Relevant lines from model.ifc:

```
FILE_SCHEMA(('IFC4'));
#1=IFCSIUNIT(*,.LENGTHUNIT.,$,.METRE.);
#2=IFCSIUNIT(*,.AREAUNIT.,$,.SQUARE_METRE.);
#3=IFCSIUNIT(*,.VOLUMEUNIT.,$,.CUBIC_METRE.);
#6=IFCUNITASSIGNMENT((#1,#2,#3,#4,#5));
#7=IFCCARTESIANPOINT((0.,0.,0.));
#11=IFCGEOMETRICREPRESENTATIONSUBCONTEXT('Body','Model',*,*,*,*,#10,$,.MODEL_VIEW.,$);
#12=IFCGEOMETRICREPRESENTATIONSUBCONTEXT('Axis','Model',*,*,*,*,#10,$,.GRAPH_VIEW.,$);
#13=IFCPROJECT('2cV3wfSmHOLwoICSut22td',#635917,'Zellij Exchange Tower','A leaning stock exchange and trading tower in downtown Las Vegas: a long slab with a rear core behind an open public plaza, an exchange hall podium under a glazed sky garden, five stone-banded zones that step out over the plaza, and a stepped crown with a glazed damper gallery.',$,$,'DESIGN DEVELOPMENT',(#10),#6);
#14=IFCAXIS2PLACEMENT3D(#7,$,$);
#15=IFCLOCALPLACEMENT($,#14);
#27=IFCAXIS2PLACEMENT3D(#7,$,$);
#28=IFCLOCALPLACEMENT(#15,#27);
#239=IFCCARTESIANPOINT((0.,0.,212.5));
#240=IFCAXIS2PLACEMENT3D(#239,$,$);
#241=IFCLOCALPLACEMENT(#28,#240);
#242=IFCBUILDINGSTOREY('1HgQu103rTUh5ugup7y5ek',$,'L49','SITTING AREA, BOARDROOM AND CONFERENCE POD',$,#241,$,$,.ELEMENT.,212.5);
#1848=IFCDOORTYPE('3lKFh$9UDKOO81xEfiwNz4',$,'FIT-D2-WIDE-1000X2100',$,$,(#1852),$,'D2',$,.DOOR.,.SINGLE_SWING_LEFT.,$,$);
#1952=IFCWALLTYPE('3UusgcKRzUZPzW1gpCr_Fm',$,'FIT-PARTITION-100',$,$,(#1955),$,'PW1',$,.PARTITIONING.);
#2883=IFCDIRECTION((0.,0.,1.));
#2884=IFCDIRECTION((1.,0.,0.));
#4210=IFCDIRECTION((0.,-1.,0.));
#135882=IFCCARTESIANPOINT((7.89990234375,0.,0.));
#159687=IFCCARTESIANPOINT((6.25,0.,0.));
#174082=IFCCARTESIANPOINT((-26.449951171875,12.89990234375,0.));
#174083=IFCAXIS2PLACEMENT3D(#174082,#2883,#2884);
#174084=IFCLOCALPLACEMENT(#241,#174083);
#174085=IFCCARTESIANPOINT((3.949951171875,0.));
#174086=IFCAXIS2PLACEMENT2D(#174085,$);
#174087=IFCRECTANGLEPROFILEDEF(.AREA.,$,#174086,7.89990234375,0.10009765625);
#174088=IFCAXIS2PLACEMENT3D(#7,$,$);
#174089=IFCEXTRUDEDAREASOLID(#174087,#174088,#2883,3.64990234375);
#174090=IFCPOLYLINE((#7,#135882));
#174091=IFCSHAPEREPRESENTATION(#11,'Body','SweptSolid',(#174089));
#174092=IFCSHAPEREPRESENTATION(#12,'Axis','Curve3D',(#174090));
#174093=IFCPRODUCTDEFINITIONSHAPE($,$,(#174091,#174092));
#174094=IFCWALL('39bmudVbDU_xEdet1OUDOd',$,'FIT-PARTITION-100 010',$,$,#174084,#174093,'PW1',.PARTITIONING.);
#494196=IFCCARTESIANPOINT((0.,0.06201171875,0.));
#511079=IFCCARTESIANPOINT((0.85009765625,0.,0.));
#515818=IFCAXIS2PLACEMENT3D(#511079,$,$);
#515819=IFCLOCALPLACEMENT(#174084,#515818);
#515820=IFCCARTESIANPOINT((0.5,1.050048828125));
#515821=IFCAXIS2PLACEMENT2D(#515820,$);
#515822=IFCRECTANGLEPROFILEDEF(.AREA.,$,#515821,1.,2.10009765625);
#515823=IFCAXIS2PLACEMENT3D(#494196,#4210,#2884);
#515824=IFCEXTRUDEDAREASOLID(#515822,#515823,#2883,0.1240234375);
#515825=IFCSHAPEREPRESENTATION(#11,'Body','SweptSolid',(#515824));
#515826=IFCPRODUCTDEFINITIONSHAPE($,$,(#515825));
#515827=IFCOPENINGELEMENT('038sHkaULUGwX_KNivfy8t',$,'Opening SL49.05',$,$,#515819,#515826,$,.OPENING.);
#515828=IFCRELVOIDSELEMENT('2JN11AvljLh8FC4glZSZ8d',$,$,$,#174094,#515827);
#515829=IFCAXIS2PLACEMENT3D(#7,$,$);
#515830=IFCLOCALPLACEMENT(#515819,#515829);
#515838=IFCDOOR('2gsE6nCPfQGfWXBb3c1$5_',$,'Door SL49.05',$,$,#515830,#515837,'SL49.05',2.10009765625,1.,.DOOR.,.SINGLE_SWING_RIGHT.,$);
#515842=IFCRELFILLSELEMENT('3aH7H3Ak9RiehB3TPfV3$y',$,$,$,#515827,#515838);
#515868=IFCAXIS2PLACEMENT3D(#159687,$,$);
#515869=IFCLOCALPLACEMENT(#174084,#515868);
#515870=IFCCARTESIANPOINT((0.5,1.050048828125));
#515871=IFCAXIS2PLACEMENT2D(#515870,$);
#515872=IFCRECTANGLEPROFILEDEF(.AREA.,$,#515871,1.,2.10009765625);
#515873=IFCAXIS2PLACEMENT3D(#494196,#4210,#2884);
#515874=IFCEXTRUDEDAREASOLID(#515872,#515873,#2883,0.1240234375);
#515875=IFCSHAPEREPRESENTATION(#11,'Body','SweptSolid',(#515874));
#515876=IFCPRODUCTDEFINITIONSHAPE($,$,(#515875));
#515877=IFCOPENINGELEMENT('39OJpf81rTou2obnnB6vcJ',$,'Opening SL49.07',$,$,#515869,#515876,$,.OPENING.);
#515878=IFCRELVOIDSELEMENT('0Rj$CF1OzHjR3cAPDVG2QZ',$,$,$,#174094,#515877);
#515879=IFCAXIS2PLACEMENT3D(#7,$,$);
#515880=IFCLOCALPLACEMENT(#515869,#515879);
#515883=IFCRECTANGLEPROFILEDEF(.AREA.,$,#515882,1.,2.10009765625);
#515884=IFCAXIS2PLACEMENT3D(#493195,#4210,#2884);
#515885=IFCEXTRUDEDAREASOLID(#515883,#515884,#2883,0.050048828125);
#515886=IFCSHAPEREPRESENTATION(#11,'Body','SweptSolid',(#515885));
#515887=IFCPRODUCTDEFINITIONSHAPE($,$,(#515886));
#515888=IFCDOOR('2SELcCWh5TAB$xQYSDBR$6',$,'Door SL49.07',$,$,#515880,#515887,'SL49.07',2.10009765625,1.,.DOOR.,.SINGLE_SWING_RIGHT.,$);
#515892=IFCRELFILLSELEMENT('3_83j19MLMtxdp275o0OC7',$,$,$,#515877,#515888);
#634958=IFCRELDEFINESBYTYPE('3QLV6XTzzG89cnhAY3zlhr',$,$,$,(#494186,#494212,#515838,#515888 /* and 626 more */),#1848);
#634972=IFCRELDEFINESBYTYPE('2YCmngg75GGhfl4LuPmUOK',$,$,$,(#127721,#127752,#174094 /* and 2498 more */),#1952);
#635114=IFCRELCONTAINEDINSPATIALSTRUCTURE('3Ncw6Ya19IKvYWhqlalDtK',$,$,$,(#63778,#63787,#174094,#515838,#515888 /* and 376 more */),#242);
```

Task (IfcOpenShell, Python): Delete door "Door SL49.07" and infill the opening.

```python
import ifcopenshell
import ifcopenshell.api.feature
import ifcopenshell.api.root
import ifcopenshell.geom
import ifcopenshell.util.shape

model = ifcopenshell.open("model.ifc")
settings = ifcopenshell.geom.settings()


def volume(element):
    """Net volume in cubic metres, openings subtracted."""
    shape = ifcopenshell.geom.create_shape(settings, element)
    return ifcopenshell.util.shape.get_volume(shape.geometry)


door = model.by_guid("2SELcCWh5TAB$xQYSDBR$6")
opening = door.FillsVoids[0].RelatingOpeningElement
wall = opening.VoidsElements[0].RelatingBuildingElement
before = volume(wall)

ifcopenshell.api.root.remove_product(model, product=door)
ifcopenshell.api.feature.remove_feature(model, feature=opening)

after = volume(wall)

print(f"wall volume {before:.3f} -> {after:.3f} m3")

model.write("model_v2.ifc")
```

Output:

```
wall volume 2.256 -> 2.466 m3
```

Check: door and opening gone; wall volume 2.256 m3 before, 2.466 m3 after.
